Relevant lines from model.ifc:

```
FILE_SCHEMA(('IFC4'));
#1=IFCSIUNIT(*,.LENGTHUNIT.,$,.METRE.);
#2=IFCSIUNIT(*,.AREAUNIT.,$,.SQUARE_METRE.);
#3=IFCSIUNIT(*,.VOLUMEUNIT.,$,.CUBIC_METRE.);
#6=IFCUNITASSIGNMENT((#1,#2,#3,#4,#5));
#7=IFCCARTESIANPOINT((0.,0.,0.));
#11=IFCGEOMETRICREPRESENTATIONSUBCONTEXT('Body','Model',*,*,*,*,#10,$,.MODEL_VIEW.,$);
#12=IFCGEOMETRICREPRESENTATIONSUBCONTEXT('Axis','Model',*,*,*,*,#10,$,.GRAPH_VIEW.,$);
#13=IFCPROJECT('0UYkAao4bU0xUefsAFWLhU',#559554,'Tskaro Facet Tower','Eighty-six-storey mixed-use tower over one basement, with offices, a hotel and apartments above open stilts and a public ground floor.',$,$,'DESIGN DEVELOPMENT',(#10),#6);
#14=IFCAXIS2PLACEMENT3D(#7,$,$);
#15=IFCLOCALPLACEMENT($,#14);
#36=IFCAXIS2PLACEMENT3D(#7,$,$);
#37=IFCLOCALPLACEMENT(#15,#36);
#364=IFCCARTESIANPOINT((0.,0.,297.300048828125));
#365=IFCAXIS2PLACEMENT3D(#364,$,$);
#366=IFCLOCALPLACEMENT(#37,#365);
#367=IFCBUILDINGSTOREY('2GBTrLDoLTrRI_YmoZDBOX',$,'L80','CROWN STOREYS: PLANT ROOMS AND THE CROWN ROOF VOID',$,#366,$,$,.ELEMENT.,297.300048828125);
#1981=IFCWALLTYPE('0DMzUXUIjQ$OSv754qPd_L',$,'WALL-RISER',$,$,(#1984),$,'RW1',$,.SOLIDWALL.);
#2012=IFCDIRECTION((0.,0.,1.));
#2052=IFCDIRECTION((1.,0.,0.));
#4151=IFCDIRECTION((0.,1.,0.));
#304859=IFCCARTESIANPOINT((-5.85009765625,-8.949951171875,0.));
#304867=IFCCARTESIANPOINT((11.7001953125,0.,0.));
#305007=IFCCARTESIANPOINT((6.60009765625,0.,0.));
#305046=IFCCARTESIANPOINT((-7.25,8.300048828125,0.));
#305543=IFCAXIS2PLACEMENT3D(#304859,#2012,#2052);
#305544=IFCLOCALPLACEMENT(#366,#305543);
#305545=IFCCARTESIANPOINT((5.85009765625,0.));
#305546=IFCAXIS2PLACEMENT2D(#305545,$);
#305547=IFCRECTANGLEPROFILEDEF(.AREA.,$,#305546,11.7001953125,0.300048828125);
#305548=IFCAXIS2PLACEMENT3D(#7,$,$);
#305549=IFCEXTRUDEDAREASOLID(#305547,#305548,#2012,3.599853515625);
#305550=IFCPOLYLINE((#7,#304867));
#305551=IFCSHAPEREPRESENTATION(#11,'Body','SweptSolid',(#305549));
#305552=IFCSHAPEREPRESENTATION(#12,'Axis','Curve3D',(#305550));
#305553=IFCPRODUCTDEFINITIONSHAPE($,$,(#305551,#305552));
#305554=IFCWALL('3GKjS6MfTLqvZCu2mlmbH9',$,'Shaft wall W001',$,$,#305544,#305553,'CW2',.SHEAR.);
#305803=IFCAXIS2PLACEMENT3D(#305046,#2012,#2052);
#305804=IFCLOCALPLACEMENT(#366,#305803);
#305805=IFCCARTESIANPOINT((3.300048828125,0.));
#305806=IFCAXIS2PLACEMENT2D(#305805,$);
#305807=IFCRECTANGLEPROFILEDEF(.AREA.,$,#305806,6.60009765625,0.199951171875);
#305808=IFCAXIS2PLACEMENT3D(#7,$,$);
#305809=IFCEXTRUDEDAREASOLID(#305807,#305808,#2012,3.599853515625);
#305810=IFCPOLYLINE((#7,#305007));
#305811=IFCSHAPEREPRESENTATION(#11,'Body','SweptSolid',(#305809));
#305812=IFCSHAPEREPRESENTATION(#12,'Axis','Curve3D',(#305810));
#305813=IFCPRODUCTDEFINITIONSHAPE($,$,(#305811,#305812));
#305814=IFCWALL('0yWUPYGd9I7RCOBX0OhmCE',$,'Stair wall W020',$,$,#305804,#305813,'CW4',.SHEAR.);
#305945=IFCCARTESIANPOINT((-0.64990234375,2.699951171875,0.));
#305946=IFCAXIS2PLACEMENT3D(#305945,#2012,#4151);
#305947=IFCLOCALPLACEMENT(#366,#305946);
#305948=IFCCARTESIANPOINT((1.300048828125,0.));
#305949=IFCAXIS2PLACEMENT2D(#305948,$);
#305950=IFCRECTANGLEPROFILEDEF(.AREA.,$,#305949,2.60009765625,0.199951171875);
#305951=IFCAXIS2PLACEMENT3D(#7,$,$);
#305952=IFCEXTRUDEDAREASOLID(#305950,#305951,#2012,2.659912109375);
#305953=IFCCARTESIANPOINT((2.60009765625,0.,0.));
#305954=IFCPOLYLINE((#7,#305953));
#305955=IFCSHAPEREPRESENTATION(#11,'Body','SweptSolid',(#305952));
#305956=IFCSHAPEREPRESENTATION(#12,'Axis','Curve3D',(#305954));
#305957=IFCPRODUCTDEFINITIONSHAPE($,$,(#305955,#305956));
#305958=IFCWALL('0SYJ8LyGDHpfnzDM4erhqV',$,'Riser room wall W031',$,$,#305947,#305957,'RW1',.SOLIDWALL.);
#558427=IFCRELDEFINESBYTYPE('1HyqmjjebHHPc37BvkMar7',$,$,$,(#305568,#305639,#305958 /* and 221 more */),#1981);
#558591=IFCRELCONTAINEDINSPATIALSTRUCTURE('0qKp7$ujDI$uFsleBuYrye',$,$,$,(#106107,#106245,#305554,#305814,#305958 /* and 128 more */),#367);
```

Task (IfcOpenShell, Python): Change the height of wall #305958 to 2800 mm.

```python
import ifcopenshell
import ifcopenshell.geom
import ifcopenshell.util.representation
import ifcopenshell.util.shape
import ifcopenshell.util.unit

model = ifcopenshell.open("model.ifc")
unit_scale = ifcopenshell.util.unit.calculate_unit_scale(model)
settings = ifcopenshell.geom.settings()


def volume(element):
    """Net volume in cubic metres, openings subtracted."""
    shape = ifcopenshell.geom.create_shape(settings, element)
    return ifcopenshell.util.shape.get_volume(shape.geometry)


wall = model.by_guid("0SYJ8LyGDHpfnzDM4erhqV")
before = volume(wall)

body = ifcopenshell.util.representation.get_representation(wall, "Model", "Body")
solid = body.Items[0]
old_height = solid.Depth
solid.Depth = 2.8 / unit_scale
after = volume(wall)

print(f"height {old_height:g} -> {solid.Depth:g}, volume {before:.3f} -> {after:.3f} m3")

model.write("model_rev.ifc")
```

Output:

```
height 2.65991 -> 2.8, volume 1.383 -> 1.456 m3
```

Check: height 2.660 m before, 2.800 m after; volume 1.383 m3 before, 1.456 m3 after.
